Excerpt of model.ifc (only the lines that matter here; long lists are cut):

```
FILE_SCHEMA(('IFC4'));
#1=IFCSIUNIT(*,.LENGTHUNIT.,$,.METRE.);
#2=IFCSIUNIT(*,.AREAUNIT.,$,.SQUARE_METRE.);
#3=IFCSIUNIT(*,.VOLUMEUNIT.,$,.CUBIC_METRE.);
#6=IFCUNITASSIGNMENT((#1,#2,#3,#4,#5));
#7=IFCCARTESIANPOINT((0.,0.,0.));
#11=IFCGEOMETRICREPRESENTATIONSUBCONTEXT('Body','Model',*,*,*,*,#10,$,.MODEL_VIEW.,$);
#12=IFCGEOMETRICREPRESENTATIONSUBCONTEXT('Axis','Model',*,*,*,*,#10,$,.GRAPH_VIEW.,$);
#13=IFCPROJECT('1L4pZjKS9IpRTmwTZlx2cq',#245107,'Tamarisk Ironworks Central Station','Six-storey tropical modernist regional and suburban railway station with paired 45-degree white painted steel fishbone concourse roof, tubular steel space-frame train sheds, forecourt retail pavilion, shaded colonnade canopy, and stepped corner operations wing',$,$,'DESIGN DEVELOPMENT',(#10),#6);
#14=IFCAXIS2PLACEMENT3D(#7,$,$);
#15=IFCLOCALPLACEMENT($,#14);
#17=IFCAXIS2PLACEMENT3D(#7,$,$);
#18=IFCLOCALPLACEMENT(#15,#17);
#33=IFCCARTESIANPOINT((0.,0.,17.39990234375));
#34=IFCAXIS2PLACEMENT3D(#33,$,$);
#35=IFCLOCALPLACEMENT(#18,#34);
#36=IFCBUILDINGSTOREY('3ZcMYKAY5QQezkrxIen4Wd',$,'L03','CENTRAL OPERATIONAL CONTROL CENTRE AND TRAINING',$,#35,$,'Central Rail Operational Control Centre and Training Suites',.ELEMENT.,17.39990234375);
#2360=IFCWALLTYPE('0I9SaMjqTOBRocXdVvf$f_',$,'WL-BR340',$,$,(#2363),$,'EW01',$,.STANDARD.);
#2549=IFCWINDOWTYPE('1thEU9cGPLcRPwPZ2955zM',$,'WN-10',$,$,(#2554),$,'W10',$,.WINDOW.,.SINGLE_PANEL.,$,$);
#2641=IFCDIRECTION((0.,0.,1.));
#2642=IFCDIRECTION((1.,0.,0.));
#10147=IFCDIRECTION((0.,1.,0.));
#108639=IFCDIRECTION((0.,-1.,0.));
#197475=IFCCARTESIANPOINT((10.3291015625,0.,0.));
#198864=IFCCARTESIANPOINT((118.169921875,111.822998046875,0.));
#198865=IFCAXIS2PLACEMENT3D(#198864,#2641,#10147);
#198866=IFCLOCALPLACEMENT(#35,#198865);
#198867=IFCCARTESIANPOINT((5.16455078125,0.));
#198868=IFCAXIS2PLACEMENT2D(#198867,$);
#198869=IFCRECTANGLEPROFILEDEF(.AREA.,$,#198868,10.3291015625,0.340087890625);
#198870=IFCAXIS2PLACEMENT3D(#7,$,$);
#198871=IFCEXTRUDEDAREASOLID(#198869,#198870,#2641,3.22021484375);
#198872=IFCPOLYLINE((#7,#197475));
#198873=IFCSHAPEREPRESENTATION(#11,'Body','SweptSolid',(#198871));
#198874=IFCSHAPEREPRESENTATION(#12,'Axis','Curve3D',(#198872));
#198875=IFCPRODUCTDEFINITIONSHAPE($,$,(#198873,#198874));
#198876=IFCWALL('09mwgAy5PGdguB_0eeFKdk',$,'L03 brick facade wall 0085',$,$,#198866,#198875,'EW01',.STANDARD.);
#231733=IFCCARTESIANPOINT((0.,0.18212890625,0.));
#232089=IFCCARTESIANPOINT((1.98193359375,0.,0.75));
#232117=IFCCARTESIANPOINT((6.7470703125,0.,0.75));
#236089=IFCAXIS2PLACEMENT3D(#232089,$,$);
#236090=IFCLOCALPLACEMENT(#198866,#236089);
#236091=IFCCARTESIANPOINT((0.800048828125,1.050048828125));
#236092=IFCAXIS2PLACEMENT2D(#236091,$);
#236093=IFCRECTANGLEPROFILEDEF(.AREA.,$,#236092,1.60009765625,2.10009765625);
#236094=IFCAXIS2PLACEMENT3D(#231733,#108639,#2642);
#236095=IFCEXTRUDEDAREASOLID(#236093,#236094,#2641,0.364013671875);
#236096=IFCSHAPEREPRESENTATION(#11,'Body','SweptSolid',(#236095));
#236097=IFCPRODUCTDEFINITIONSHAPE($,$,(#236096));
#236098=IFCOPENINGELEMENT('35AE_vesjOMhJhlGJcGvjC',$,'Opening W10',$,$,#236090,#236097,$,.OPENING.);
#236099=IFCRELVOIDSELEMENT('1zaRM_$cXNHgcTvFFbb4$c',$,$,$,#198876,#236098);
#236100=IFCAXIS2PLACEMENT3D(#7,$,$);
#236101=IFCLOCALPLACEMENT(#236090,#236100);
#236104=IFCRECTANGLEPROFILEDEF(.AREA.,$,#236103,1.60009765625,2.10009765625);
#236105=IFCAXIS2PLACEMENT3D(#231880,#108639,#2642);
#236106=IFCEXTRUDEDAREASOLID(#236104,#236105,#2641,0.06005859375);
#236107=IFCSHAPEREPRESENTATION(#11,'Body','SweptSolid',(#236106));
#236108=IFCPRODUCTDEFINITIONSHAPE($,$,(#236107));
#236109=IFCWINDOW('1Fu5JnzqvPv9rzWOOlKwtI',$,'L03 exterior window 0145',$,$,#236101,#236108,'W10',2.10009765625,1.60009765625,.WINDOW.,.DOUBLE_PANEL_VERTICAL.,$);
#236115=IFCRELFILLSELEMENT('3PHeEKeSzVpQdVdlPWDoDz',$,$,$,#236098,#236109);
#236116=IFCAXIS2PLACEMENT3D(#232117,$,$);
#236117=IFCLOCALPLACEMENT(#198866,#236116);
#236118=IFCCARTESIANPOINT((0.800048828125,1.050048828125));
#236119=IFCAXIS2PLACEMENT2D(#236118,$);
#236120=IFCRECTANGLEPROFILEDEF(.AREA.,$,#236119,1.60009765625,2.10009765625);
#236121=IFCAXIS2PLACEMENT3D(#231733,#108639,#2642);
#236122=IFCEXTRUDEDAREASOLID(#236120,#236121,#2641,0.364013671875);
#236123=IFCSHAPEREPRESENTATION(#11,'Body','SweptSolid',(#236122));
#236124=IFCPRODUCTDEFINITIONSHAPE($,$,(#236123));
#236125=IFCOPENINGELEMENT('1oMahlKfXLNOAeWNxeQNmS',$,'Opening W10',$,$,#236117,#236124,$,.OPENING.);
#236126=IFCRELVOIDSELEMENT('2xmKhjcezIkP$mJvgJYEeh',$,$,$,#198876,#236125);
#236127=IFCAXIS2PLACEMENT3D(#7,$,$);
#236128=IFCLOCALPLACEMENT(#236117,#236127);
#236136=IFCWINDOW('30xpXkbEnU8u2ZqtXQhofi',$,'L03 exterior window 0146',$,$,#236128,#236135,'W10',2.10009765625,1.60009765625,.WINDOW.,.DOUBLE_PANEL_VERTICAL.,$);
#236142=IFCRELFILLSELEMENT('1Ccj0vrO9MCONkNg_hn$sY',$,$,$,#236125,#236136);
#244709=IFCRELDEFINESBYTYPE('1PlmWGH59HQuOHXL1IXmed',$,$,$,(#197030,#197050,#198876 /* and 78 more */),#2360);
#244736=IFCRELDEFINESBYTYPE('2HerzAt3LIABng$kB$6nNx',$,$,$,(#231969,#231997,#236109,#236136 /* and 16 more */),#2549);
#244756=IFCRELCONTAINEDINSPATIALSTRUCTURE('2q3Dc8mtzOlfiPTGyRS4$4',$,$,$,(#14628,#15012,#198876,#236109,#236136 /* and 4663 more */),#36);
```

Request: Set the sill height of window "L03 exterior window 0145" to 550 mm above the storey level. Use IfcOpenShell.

```python
import numpy as np
import ifcopenshell
import ifcopenshell.api.geometry
import ifcopenshell.geom
import ifcopenshell.util.element
import ifcopenshell.util.placement
import ifcopenshell.util.shape
import ifcopenshell.util.unit

model = ifcopenshell.open("model.ifc")
unit_scale = ifcopenshell.util.unit.calculate_unit_scale(model)

window = model.by_guid("1Fu5JnzqvPv9rzWOOlKwtI")
opening = window.FillsVoids[0].RelatingOpeningElement
storey = ifcopenshell.util.element.get_container(window, ifc_class="IfcBuildingStorey")
level = ifcopenshell.util.placement.get_local_placement(storey.ObjectPlacement)[2, 3]

# The opening's origin need not be at the sill, so measure its lowest point.
shape = ifcopenshell.geom.create_shape(ifcopenshell.geom.settings(), opening)
bottom = ifcopenshell.util.shape.get_shape_bottom_elevation(shape, shape.geometry) / unit_scale
dz = level + 0.55 / unit_scale - bottom

shift = np.array([0.0, 0.0, dz])
# The window is placed relative to its opening, so it follows when the opening moves.
matrix = ifcopenshell.util.placement.get_local_placement(opening.ObjectPlacement)
matrix[:3, 3] += shift
ifcopenshell.api.geometry.edit_object_placement(
    model, product=opening, matrix=matrix, is_si=False, should_transform_children=True
)

print(f"moved by {dz * unit_scale:+.3f} m")

model.write("model_v2.ifc")
```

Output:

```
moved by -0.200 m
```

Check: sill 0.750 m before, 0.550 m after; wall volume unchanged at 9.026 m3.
